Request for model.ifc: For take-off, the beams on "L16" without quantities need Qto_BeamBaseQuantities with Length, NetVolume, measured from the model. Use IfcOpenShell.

First a look at what the model holds.

```python
import ifcopenshell
import ifcopenshell.util.element
import ifcopenshell.util.unit

model = ifcopenshell.open("model.ifc")
print(model.schema)
for unit_type in ("LENGTHUNIT", "AREAUNIT", "VOLUMEUNIT"):
    print(unit_type, ifcopenshell.util.unit.calculate_unit_scale(model, unit_type))
storey = next(s for s in model.by_type("IfcBuildingStorey") if s.Name == "L16")
beams = [e for e in ifcopenshell.util.element.get_decomposition(storey) if e.is_a("IfcBeam")]
for e in sorted(beams, key=lambda e: e.id()):
    print(e.id(), e.is_a(), e.Name, list(ifcopenshell.util.element.get_psets(e, qtos_only=True)), sep=" | ")
```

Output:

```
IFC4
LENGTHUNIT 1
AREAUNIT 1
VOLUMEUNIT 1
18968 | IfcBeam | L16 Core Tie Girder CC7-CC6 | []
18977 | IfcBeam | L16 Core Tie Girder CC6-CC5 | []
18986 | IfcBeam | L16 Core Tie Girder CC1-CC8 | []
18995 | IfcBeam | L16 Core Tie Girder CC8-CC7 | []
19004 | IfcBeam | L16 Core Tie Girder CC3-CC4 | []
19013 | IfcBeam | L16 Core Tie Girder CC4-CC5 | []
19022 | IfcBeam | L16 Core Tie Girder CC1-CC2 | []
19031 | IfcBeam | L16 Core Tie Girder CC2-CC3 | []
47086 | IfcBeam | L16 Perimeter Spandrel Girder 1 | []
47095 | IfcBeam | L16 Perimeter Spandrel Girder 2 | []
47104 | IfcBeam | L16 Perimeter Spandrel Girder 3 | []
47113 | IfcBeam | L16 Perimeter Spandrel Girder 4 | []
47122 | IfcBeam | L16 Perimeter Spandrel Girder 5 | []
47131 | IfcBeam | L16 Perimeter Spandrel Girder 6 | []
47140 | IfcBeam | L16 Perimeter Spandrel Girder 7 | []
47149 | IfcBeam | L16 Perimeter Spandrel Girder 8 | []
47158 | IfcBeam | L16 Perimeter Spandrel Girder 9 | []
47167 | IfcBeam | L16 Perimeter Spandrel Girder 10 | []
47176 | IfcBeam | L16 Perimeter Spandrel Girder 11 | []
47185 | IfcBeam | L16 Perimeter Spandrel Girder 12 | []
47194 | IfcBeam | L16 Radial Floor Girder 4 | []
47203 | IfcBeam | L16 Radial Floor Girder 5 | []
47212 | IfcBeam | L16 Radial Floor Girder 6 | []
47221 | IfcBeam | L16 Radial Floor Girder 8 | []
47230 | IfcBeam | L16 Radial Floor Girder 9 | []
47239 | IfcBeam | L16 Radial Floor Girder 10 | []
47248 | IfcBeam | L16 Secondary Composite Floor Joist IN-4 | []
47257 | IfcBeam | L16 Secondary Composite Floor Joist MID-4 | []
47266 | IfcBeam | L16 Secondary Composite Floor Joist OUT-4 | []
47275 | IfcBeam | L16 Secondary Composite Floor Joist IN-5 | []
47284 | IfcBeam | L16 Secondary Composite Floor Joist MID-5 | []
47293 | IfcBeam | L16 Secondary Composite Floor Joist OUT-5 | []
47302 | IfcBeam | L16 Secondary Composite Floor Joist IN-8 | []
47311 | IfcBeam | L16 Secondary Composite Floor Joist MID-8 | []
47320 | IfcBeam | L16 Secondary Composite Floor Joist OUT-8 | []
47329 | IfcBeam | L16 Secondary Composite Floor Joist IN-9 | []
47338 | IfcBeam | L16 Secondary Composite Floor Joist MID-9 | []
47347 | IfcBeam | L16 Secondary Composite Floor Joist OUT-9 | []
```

```python
import ifcopenshell
import ifcopenshell.api.pset
import ifcopenshell.geom
import ifcopenshell.util.element
import ifcopenshell.util.shape
import ifcopenshell.util.unit

model = ifcopenshell.open("model.ifc")
unit_scale = ifcopenshell.util.unit.calculate_unit_scale(model)
volume_scale = ifcopenshell.util.unit.calculate_unit_scale(model, "VOLUMEUNIT")
settings = ifcopenshell.geom.settings()

storey = next(s for s in model.by_type("IfcBuildingStorey") if s.Name == "L16")
beams = [e for e in ifcopenshell.util.element.get_decomposition(storey) if e.is_a("IfcBeam")]

for e in sorted(beams, key=lambda e: e.id()):
    if ifcopenshell.util.element.get_psets(e, qtos_only=True, should_inherit=False):
        continue
    # Geometry comes back in metres, in the element's own axes.
    shape = ifcopenshell.geom.create_shape(settings, e)
    values = {
        "Length": ifcopenshell.util.shape.get_max_xyz(shape.geometry) / unit_scale,
        "NetVolume": ifcopenshell.util.shape.get_volume(shape.geometry) / volume_scale,
    }
    qto = ifcopenshell.api.pset.add_qto(model, product=e, name="Qto_BeamBaseQuantities")
    ifcopenshell.api.pset.edit_qto(model, qto=qto, properties=values)
    print(e.id(), {k: round(v, 3) for k, v in values.items()})

model.write("model-out.ifc")
```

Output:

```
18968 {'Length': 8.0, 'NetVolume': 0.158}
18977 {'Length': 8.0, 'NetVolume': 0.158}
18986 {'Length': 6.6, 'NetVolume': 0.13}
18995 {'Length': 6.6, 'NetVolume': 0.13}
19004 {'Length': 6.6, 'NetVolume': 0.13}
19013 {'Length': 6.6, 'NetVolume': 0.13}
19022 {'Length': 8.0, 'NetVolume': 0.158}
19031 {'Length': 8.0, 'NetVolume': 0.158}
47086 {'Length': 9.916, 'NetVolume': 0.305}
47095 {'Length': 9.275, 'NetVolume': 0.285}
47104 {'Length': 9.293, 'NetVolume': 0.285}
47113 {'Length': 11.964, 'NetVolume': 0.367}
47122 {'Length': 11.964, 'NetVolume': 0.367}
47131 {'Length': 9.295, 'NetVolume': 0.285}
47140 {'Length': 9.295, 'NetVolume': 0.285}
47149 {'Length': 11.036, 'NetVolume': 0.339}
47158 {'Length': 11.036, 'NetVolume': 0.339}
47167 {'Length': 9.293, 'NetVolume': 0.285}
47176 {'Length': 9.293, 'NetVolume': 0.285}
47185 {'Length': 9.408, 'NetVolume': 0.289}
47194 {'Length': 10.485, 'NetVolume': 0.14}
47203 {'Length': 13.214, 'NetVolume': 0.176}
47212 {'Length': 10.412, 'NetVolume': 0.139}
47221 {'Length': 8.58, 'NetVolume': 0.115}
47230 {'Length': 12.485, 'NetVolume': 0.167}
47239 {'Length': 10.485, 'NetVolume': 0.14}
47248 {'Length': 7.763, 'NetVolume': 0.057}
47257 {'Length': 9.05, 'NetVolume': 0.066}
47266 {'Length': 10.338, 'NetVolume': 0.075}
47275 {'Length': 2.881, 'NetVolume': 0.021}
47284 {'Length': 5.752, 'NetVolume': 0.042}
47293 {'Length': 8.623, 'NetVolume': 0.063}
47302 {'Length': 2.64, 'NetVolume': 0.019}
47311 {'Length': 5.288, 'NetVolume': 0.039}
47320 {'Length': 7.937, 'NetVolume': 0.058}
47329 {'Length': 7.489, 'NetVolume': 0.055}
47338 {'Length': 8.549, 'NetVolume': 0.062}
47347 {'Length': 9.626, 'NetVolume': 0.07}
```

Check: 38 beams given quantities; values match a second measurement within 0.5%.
